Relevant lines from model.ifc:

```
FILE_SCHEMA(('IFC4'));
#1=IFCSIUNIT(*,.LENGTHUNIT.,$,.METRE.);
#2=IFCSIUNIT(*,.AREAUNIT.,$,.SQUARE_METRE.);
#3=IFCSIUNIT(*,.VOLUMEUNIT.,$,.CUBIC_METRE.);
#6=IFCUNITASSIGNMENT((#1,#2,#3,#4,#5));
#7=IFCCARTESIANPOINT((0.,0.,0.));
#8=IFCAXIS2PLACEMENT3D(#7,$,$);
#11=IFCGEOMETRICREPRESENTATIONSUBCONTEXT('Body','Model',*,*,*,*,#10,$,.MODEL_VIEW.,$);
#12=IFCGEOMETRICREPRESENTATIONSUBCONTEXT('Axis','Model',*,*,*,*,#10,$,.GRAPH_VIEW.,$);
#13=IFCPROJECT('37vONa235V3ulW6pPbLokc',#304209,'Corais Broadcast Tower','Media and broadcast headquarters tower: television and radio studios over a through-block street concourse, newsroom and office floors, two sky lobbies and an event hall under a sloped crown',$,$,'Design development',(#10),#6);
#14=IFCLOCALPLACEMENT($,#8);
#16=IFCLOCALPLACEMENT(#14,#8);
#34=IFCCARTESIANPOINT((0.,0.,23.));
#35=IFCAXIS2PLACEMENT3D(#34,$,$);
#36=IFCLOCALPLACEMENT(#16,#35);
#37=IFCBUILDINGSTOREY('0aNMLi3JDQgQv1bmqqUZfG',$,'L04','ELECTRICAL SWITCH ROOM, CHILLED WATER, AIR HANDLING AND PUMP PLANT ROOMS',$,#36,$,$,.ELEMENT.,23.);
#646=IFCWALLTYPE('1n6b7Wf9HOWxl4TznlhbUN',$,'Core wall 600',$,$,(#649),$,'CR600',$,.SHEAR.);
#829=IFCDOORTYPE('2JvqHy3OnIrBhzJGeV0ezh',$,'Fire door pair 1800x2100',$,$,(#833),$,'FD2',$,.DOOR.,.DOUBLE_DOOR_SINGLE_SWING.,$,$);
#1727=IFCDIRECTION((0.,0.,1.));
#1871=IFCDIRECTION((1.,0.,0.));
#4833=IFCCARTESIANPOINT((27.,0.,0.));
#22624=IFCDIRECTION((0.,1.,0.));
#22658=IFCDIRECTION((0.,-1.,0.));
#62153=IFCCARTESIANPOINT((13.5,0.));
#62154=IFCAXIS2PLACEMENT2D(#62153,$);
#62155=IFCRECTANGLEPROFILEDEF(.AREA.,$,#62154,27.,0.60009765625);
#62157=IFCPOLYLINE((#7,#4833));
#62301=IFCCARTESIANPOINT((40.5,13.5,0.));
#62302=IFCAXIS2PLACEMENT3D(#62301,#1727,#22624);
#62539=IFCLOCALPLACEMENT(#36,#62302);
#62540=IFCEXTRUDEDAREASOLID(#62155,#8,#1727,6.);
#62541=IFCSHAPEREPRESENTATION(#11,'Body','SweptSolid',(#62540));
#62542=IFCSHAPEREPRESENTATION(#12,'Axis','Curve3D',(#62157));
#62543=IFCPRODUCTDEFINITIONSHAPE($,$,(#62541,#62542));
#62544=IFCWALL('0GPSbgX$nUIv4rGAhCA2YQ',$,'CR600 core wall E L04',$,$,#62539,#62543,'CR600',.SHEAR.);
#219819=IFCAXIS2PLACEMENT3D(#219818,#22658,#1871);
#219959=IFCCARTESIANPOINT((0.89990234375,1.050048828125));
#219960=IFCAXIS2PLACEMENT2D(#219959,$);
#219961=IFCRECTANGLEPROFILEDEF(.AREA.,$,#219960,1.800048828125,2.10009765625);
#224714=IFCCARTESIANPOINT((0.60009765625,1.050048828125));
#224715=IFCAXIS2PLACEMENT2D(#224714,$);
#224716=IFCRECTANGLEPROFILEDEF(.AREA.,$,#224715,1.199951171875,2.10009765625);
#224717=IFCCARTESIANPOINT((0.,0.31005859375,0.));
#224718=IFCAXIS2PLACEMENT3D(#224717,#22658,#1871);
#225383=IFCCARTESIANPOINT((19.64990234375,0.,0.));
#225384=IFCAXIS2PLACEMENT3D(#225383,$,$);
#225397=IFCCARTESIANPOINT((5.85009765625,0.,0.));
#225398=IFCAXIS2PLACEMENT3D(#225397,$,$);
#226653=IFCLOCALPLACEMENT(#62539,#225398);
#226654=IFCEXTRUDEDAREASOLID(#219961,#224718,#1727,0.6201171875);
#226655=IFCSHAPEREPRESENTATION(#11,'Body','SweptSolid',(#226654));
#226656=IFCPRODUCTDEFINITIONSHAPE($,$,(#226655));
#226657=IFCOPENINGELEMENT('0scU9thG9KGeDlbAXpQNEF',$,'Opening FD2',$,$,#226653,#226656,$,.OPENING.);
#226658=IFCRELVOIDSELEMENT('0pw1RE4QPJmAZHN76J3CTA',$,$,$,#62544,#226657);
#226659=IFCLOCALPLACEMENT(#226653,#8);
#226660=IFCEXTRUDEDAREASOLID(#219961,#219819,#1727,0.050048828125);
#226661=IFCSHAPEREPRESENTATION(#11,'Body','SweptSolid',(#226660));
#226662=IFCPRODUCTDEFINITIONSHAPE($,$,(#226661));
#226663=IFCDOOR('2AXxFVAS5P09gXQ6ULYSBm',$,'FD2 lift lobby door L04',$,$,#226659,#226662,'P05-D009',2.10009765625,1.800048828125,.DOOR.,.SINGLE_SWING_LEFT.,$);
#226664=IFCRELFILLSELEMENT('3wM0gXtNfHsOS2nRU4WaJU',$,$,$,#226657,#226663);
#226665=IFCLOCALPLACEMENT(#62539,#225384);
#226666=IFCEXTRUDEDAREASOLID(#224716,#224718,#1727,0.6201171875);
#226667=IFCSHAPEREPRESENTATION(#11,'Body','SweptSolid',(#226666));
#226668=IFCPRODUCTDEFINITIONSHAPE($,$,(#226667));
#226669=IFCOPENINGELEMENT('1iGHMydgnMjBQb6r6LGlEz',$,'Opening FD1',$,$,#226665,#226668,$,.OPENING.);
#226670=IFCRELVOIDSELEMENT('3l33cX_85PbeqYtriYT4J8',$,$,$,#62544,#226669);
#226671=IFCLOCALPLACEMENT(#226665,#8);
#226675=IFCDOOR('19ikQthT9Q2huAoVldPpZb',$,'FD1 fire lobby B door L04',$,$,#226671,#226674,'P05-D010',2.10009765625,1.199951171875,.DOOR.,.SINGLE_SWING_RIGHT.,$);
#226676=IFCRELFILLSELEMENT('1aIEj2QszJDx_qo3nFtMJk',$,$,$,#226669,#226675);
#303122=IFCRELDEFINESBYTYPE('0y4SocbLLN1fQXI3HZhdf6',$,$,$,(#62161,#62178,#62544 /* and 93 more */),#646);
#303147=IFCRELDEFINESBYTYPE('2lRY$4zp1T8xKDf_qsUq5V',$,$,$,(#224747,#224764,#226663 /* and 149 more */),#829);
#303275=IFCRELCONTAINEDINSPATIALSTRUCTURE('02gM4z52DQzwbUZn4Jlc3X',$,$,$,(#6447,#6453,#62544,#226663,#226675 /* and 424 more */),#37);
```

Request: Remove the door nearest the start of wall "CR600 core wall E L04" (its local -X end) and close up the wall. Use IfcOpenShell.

```python
import ifcopenshell
import ifcopenshell.api.feature
import ifcopenshell.api.root
import ifcopenshell.geom
import ifcopenshell.util.shape

model = ifcopenshell.open("model.ifc")
settings = ifcopenshell.geom.settings()


def volume(element):
    """Net volume in cubic metres, openings subtracted."""
    shape = ifcopenshell.geom.create_shape(settings, element)
    return ifcopenshell.util.shape.get_volume(shape.geometry)


door = model.by_guid("2AXxFVAS5P09gXQ6ULYSBm")
opening = door.FillsVoids[0].RelatingOpeningElement
wall = opening.VoidsElements[0].RelatingBuildingElement
before = volume(wall)

ifcopenshell.api.root.remove_product(model, product=door)
ifcopenshell.api.feature.remove_feature(model, feature=opening)

after = volume(wall)

print(f"wall volume {before:.3f} -> {after:.3f} m3")

model.write("model-out.ifc")
```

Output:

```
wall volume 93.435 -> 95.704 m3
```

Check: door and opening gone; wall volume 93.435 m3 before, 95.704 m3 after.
